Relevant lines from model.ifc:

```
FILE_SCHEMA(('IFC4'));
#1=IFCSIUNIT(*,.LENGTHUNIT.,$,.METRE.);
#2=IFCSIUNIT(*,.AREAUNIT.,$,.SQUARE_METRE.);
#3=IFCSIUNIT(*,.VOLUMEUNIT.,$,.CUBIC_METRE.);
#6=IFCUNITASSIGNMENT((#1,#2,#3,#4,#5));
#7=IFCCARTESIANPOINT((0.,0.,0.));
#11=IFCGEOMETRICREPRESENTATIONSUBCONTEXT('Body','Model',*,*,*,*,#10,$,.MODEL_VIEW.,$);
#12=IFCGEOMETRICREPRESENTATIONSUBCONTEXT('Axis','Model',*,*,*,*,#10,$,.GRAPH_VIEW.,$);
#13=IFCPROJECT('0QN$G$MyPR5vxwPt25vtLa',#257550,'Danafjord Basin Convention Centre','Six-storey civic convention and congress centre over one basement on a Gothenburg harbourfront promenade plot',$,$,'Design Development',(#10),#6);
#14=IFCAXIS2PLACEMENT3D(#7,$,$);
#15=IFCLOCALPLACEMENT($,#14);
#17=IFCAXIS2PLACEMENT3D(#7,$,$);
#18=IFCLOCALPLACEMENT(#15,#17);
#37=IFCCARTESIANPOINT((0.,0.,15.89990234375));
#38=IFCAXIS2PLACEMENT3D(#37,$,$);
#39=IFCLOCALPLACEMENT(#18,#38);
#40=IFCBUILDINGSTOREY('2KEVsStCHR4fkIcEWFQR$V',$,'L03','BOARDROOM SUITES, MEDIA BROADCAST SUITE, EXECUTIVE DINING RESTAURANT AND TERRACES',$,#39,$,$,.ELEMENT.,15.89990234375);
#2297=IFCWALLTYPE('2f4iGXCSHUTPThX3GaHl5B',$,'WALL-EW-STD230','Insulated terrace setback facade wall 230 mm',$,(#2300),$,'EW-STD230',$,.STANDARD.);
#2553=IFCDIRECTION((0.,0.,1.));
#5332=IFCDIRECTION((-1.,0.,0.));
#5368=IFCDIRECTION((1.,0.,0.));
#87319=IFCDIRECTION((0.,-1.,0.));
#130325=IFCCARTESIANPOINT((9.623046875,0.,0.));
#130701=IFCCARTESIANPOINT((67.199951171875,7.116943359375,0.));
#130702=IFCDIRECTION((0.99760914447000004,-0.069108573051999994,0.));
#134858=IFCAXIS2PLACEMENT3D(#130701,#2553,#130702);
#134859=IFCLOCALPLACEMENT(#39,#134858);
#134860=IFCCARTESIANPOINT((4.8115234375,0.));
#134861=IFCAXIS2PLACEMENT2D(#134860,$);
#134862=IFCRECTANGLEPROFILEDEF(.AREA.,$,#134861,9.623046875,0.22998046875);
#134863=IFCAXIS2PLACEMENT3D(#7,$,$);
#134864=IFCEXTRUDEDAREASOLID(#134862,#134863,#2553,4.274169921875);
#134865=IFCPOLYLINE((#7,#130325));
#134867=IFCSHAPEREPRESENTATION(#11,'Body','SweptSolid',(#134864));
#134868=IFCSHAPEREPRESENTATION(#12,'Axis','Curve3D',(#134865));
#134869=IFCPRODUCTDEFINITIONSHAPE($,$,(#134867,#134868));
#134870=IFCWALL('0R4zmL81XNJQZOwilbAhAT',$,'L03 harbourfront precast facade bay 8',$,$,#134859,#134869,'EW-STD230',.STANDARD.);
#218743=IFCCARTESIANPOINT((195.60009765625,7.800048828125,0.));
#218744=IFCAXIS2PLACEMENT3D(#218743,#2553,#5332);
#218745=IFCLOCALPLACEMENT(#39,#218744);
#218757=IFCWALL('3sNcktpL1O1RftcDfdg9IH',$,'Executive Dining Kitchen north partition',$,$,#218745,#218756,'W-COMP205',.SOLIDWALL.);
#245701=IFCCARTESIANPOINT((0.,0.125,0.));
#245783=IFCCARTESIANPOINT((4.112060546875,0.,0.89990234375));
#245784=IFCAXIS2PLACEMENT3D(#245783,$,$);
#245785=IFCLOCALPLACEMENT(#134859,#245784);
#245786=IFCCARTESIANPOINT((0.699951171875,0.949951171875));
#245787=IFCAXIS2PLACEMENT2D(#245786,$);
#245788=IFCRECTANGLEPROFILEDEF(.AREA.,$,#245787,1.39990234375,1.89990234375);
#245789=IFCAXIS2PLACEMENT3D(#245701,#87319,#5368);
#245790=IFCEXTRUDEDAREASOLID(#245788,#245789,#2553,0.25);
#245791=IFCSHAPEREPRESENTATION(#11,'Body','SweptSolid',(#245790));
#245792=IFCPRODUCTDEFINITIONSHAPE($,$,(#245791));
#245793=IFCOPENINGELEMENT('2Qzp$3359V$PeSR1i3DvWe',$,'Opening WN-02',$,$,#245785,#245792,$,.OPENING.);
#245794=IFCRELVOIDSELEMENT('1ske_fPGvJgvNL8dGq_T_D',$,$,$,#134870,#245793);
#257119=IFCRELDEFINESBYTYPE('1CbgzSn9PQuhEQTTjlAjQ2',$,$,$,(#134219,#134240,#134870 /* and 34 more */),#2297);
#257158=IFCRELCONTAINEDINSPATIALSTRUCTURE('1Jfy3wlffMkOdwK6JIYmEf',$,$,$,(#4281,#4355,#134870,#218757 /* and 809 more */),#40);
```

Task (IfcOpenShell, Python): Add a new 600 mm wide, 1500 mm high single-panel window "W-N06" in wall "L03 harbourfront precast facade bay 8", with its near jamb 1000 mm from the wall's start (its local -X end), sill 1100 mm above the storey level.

```python
import numpy as np
import ifcopenshell
import ifcopenshell.api.feature
import ifcopenshell.api.geometry
import ifcopenshell.api.root
import ifcopenshell.api.spatial
import ifcopenshell.geom
import ifcopenshell.util.element
import ifcopenshell.util.placement
import ifcopenshell.util.representation
import ifcopenshell.util.shape
import ifcopenshell.util.unit

model = ifcopenshell.open("model.ifc")
unit_scale = ifcopenshell.util.unit.calculate_unit_scale(model)
settings = ifcopenshell.geom.settings()


def volume(element):
    """Net volume in cubic metres, openings subtracted."""
    shape = ifcopenshell.geom.create_shape(settings, element)
    return ifcopenshell.util.shape.get_volume(shape.geometry)


wall = model.by_guid("0R4zmL81XNJQZOwilbAhAT")
storey = ifcopenshell.util.element.get_container(wall, ifc_class="IfcBuildingStorey")
context = ifcopenshell.util.representation.get_context(model, "Model", "Body", "MODEL_VIEW")
before = volume(wall)

width, height, from_end, sill = 0.6, 1.5, 1, 1.1  # metres

# The wall runs along its own X axis, and the end named is its -X end.
wall_shape = ifcopenshell.geom.create_shape(settings, wall)
x, y, z = ifcopenshell.util.shape.get_vertices(wall_shape.geometry).T
start = x.min() + from_end
face, thickness = float(y.min()), float(y.max() - y.min())
wall_matrix = ifcopenshell.util.placement.get_local_placement(wall.ObjectPlacement)
level = ifcopenshell.util.placement.get_local_placement(storey.ObjectPlacement)[2, 3]


def in_wall(x, y):
    """Placement at x, y metres in the wall's axes, at sill height."""
    matrix = wall_matrix.copy()
    matrix[:, 3] = wall_matrix @ np.array([x / unit_scale, y / unit_scale, 0.0, 1.0])
    matrix[2, 3] = level + sill / unit_scale
    return matrix


# Opening: a box that overshoots both wall faces by 50 mm.
opening = ifcopenshell.api.root.create_entity(model, ifc_class="IfcOpeningElement", predefined_type="OPENING")
box = ifcopenshell.api.geometry.add_wall_representation(
    model, context=context, length=width, height=height, thickness=thickness + 0.1
)
ifcopenshell.api.geometry.assign_representation(model, product=opening, representation=box)
ifcopenshell.api.geometry.edit_object_placement(model, product=opening, matrix=in_wall(start, face - 0.05), is_si=False)
ifcopenshell.api.feature.add_feature(model, feature=opening, element=wall)

window = ifcopenshell.api.root.create_entity(model, ifc_class="IfcWindow", name="W-N06", predefined_type="WINDOW")
window.OverallWidth, window.OverallHeight = width / unit_scale, height / unit_scale
window.PartitioningType = "SINGLE_PANEL"
body = ifcopenshell.api.geometry.add_window_representation(
    model,
    context=context,
    overall_width=window.OverallWidth,
    overall_height=window.OverallHeight,
    partition_type="SINGLE_PANEL",
)
ifcopenshell.api.geometry.assign_representation(model, product=window, representation=body)
ifcopenshell.api.spatial.assign_container(model, products=[window], relating_structure=storey)
ifcopenshell.api.feature.add_filling(model, opening=opening, element=window)

# Centre the window in the wall's thickness.
ifcopenshell.api.geometry.edit_object_placement(model, product=window, matrix=in_wall(start, face), is_si=False)
window_shape = ifcopenshell.geom.create_shape(settings, window)
depth = ifcopenshell.util.shape.get_vertices(window_shape.geometry)[:, 1]
offset = face + thickness / 2 - (depth.min() + depth.max()) / 2
ifcopenshell.api.geometry.edit_object_placement(model, product=window, matrix=in_wall(start, offset), is_si=False)

after = volume(wall)

print(f"wall volume {before:.3f} -> {after:.3f} m3")

model.write("model_rev.ifc")
```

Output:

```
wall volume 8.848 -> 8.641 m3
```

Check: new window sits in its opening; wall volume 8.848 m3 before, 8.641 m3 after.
